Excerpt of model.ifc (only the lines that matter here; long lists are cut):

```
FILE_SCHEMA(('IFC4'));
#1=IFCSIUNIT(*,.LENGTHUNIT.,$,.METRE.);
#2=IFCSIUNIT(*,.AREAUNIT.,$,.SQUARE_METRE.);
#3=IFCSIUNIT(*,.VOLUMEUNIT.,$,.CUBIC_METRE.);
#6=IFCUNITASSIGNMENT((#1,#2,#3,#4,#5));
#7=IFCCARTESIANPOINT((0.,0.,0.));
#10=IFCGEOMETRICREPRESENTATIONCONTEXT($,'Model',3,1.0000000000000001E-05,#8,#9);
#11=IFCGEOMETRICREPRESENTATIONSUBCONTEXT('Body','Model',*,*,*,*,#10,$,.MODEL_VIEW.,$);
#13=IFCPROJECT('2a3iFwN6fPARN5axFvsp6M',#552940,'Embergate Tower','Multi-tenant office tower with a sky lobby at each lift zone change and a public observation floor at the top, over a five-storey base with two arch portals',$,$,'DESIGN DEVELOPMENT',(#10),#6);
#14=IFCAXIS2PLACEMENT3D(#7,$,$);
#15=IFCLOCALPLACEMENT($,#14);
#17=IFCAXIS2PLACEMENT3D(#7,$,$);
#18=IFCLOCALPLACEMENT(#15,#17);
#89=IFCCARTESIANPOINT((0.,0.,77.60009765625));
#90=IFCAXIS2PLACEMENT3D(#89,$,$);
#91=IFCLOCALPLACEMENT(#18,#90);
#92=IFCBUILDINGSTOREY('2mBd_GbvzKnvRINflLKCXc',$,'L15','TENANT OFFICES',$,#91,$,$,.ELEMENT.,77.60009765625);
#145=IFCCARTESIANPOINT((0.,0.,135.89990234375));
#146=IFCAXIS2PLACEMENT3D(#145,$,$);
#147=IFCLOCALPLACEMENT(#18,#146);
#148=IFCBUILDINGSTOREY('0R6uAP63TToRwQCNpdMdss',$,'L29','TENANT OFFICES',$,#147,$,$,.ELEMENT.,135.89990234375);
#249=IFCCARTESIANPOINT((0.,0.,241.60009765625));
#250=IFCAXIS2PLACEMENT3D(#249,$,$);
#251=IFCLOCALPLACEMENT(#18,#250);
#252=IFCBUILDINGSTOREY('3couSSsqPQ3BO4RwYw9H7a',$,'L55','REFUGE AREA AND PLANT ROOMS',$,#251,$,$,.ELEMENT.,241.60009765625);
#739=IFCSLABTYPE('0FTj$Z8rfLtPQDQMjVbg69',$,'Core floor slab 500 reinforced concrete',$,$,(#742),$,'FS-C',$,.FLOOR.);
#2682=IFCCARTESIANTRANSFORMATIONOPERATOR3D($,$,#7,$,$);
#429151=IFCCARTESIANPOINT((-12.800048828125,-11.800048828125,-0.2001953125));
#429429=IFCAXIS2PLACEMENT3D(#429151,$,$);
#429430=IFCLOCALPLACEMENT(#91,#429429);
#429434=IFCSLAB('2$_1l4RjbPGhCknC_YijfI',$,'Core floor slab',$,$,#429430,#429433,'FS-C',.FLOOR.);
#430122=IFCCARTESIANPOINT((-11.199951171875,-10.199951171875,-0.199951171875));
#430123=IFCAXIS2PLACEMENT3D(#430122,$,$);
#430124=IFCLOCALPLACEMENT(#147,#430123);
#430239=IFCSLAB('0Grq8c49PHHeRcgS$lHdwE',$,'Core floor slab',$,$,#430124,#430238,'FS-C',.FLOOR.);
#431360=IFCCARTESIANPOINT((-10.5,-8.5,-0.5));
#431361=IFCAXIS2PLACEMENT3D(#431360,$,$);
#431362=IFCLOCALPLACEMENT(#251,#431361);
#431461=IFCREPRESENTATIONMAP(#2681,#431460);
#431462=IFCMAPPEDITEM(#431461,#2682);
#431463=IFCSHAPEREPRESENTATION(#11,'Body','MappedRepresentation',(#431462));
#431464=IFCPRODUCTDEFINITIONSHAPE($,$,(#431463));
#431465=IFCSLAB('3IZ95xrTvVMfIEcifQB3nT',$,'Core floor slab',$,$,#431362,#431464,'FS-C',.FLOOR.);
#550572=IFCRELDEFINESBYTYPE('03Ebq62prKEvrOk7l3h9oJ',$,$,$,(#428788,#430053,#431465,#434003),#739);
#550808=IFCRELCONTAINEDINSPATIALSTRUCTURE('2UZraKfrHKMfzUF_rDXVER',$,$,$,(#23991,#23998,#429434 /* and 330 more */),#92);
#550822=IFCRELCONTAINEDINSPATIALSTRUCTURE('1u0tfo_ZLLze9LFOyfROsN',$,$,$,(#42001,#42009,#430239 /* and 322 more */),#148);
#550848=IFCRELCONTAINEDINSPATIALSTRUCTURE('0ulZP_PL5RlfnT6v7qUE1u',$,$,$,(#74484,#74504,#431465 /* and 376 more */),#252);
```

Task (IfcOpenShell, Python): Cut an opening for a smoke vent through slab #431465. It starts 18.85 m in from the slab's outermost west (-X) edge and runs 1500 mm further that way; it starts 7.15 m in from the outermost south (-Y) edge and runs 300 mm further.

```python
import numpy as np
import ifcopenshell
import ifcopenshell.api.feature
import ifcopenshell.api.geometry
import ifcopenshell.api.root
import ifcopenshell.geom
import ifcopenshell.util.placement
import ifcopenshell.util.representation
import ifcopenshell.util.shape
import ifcopenshell.util.unit

model = ifcopenshell.open("model.ifc")
unit_scale = ifcopenshell.util.unit.calculate_unit_scale(model)
settings = ifcopenshell.geom.settings()


def volume(element):
    """Net volume in cubic metres, openings subtracted."""
    shape = ifcopenshell.geom.create_shape(settings, element)
    return ifcopenshell.util.shape.get_volume(shape.geometry)


slab = model.by_guid("3IZ95xrTvVMfIEcifQB3nT")
before = volume(slab)

# Extent in the slab's own axes, in metres. The edges named are its -X and -Y sides.
slab_shape = ifcopenshell.geom.create_shape(settings, slab)
vertices = ifcopenshell.util.shape.get_vertices(slab_shape.geometry)
x_min, y_min, bottom = vertices.min(axis=0)
top = vertices[:, 2].max()

opening = ifcopenshell.api.root.create_entity(model, ifc_class="IfcOpeningElement", name="Smoke vent opening", predefined_type="OPENING")
context = ifcopenshell.util.representation.get_context(model, "Model", "Body", "MODEL_VIEW")
width, depth = 1.5, 0.3
outline = [(0.0, 0.0), (width, 0.0), (width, depth), (0.0, depth), (0.0, 0.0)]
# Overshoot both faces by 50 mm so the cut is clean.
shape = ifcopenshell.api.geometry.add_slab_representation(
    model, context=context, depth=top - bottom + 0.1, polyline=outline
)
ifcopenshell.api.geometry.assign_representation(model, product=opening, representation=shape)

matrix = ifcopenshell.util.placement.get_local_placement(slab.ObjectPlacement)
matrix[:, 3] = matrix @ np.append(np.array([x_min + 18.85, y_min + 7.15, bottom - 0.05]) / unit_scale, 1.0)
ifcopenshell.api.geometry.edit_object_placement(model, product=opening, matrix=matrix, is_si=False)
ifcopenshell.api.feature.add_feature(model, feature=opening, element=slab)

after = volume(slab)

print(f"slab volume {before:.3f} -> {after:.3f} m3")

model.write("model_updated.ifc")
```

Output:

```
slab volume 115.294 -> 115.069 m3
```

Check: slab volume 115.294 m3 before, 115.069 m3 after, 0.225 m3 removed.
